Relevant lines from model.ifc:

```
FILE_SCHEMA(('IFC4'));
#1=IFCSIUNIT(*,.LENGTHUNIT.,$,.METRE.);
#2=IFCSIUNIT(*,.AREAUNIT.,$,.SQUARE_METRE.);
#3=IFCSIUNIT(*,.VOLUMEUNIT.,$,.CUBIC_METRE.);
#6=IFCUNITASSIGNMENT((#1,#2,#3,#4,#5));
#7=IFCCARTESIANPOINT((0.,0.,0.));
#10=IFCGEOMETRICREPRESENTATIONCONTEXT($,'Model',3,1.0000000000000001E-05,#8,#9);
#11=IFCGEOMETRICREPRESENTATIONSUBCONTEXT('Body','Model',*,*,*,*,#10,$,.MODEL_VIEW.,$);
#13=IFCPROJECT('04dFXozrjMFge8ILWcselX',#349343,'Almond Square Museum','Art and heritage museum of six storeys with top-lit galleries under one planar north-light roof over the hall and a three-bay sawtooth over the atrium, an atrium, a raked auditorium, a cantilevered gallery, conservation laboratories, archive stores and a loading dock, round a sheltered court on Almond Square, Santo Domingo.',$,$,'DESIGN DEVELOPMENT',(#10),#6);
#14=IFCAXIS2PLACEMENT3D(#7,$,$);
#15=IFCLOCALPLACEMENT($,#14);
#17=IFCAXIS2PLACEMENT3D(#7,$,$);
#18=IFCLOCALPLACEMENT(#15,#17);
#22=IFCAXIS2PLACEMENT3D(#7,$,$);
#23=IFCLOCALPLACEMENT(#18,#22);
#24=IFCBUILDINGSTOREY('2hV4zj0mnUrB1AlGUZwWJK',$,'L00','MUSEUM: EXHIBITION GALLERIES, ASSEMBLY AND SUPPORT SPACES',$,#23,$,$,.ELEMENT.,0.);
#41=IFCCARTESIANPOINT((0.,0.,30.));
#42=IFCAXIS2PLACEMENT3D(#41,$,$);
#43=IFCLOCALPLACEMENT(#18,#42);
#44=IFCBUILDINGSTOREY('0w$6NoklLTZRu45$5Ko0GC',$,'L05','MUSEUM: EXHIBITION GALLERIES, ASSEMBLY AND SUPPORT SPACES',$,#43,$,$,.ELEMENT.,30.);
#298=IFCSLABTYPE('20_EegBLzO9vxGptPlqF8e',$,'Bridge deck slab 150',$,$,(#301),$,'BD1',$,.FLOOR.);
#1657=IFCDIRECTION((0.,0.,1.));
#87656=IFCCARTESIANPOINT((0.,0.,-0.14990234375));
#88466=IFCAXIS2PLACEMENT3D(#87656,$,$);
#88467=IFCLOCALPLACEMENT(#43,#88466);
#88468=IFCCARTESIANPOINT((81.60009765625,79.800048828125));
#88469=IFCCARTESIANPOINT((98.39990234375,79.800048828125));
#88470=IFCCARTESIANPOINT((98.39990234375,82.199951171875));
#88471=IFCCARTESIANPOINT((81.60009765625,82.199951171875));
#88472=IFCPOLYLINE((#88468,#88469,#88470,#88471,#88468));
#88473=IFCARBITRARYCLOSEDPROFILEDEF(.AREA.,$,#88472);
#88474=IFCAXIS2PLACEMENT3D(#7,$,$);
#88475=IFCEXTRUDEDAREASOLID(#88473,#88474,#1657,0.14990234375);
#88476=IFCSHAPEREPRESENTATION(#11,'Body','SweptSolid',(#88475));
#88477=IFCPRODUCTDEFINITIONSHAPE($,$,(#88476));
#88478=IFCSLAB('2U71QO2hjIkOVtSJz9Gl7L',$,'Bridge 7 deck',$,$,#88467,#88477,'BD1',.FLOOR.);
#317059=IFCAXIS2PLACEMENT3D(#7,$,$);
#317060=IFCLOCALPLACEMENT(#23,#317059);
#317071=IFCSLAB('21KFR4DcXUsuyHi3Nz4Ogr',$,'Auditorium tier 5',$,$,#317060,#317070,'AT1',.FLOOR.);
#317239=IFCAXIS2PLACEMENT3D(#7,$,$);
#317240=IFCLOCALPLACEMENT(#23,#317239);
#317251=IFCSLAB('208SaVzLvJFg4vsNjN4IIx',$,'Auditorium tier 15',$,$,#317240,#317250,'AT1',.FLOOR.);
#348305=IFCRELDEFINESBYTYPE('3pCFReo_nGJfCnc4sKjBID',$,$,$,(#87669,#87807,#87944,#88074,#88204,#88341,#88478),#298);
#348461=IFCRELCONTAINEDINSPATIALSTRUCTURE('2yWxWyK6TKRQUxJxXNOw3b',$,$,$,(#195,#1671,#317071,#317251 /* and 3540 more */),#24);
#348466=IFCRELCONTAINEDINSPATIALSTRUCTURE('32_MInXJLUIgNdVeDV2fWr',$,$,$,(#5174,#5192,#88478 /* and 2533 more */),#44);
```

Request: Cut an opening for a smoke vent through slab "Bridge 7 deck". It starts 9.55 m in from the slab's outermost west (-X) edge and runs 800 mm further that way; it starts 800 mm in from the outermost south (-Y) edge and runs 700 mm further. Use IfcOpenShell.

```python
import numpy as np
import ifcopenshell
import ifcopenshell.api.feature
import ifcopenshell.api.geometry
import ifcopenshell.api.root
import ifcopenshell.geom
import ifcopenshell.util.placement
import ifcopenshell.util.representation
import ifcopenshell.util.shape
import ifcopenshell.util.unit

model = ifcopenshell.open("model.ifc")
unit_scale = ifcopenshell.util.unit.calculate_unit_scale(model)
settings = ifcopenshell.geom.settings()


def volume(element):
    """Net volume in cubic metres, openings subtracted."""
    shape = ifcopenshell.geom.create_shape(settings, element)
    return ifcopenshell.util.shape.get_volume(shape.geometry)


slab = model.by_guid("2U71QO2hjIkOVtSJz9Gl7L")
before = volume(slab)

# Extent in the slab's own axes, in metres. The edges named are its -X and -Y sides.
slab_shape = ifcopenshell.geom.create_shape(settings, slab)
vertices = ifcopenshell.util.shape.get_vertices(slab_shape.geometry)
x_min, y_min, bottom = vertices.min(axis=0)
top = vertices[:, 2].max()

opening = ifcopenshell.api.root.create_entity(model, ifc_class="IfcOpeningElement", name="Smoke vent opening", predefined_type="OPENING")
context = ifcopenshell.util.representation.get_context(model, "Model", "Body", "MODEL_VIEW")
width, depth = 0.8, 0.7
outline = [(0.0, 0.0), (width, 0.0), (width, depth), (0.0, depth), (0.0, 0.0)]
# Overshoot both faces by 50 mm so the cut is clean.
shape = ifcopenshell.api.geometry.add_slab_representation(
    model, context=context, depth=top - bottom + 0.1, polyline=outline
)
ifcopenshell.api.geometry.assign_representation(model, product=opening, representation=shape)

matrix = ifcopenshell.util.placement.get_local_placement(slab.ObjectPlacement)
matrix[:, 3] = matrix @ np.append(np.array([x_min + 9.55, y_min + 0.8, bottom - 0.05]) / unit_scale, 1.0)
ifcopenshell.api.geometry.edit_object_placement(model, product=opening, matrix=matrix, is_si=False)
ifcopenshell.api.feature.add_feature(model, feature=opening, element=slab)

after = volume(slab)

print(f"slab volume {before:.3f} -> {after:.3f} m3")

model.write("model_rev.ifc")
```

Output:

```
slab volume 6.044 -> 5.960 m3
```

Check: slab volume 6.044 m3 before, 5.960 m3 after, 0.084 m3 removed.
